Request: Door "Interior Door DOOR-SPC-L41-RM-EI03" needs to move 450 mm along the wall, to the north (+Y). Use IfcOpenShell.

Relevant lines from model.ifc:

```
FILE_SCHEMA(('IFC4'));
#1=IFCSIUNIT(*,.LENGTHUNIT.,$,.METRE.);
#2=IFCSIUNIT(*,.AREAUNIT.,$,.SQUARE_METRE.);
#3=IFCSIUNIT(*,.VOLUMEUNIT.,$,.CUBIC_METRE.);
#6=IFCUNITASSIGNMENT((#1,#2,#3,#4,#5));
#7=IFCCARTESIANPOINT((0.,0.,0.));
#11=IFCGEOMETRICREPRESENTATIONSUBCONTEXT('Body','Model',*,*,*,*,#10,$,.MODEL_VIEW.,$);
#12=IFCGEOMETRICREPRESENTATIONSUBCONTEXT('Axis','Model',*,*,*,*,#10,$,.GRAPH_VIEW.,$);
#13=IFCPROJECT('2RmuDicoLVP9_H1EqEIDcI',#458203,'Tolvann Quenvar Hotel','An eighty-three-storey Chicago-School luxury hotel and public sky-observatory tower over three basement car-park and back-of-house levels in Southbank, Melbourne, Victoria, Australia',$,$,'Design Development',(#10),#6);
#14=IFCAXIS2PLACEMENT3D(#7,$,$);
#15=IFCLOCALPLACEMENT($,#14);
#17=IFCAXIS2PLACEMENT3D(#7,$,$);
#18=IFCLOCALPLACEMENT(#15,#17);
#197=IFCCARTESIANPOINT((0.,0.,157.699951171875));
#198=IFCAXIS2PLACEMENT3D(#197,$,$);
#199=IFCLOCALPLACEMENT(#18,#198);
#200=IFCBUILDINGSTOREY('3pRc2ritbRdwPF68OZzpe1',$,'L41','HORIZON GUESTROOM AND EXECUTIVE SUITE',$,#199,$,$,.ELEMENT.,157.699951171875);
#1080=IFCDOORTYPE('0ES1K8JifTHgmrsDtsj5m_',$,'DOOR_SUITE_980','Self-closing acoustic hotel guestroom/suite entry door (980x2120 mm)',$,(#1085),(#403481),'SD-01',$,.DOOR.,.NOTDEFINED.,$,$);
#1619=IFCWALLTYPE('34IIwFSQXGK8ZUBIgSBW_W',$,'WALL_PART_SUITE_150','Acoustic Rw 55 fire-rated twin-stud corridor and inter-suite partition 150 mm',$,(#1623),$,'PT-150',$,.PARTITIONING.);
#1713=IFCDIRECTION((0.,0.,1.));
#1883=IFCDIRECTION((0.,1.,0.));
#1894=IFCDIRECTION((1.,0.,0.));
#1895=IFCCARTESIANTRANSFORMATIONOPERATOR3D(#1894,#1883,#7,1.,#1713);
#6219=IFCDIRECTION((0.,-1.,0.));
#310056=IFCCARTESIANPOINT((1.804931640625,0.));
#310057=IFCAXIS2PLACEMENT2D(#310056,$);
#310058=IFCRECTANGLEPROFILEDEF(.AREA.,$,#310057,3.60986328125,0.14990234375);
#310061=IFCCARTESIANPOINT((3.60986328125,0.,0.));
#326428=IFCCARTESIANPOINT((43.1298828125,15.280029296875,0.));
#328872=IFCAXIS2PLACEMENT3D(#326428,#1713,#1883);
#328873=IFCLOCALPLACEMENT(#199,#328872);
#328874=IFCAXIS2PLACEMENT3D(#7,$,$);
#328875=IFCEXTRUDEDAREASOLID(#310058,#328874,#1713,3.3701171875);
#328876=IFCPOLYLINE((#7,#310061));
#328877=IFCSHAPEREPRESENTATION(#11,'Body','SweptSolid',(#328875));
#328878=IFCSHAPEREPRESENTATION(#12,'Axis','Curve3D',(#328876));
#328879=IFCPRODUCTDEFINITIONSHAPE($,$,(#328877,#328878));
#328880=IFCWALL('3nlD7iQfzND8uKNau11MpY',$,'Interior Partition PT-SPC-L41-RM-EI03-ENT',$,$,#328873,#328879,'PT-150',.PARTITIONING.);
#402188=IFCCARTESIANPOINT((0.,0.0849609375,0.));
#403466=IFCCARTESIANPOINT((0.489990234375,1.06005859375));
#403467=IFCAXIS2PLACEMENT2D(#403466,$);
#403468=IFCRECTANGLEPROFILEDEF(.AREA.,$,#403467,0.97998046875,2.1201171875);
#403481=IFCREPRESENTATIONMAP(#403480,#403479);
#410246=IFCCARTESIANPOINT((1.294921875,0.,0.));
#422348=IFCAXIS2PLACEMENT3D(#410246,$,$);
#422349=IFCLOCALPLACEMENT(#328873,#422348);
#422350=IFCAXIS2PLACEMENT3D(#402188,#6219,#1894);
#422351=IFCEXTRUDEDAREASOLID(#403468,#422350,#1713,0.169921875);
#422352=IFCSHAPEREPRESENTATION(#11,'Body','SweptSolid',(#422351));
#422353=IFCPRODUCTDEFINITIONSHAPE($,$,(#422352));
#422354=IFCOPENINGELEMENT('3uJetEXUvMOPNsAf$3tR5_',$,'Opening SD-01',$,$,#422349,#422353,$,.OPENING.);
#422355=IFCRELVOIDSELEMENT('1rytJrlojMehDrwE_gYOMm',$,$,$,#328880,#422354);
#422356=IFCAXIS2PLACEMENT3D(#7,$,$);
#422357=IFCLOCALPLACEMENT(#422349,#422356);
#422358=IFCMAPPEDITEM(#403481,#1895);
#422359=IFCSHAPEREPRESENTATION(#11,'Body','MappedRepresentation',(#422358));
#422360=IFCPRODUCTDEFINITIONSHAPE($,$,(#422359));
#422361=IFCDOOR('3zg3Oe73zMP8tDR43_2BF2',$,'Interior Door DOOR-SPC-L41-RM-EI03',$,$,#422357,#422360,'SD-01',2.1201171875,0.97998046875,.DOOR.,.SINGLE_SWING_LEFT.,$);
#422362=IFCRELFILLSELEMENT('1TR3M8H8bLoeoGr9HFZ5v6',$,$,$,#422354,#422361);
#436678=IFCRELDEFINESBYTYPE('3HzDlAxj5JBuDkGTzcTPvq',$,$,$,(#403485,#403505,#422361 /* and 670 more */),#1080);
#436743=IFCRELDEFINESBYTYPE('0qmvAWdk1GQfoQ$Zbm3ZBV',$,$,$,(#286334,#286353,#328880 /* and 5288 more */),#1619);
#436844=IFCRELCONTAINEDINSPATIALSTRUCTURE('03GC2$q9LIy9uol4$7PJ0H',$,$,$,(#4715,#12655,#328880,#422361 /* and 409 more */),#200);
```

```python
import ifcopenshell
import ifcopenshell.api.geometry
import ifcopenshell.util.placement
import ifcopenshell.util.unit

model = ifcopenshell.open("model.ifc")
unit_scale = ifcopenshell.util.unit.calculate_unit_scale(model)

door = model.by_id(422361)
opening = door.FillsVoids[0].RelatingOpeningElement
wall = opening.VoidsElements[0].RelatingBuildingElement

wall_matrix = ifcopenshell.util.placement.get_local_placement(wall.ObjectPlacement)
shift = wall_matrix[:3, 0] * 0.45 / unit_scale
before = ifcopenshell.util.placement.get_local_placement(door.ObjectPlacement)[:3, 3].copy()

# The door is placed relative to its opening, so it follows when the opening moves.
matrix = ifcopenshell.util.placement.get_local_placement(opening.ObjectPlacement)
matrix[:3, 3] += shift
ifcopenshell.api.geometry.edit_object_placement(
    model, product=opening, matrix=matrix, is_si=False, should_transform_children=True
)

after = ifcopenshell.util.placement.get_local_placement(door.ObjectPlacement)[:3, 3]
print("door moved by", (after - before).round(3) + 0.0)

model.write("model_updated.ifc")
```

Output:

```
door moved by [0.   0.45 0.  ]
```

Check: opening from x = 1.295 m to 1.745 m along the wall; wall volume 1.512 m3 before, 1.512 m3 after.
